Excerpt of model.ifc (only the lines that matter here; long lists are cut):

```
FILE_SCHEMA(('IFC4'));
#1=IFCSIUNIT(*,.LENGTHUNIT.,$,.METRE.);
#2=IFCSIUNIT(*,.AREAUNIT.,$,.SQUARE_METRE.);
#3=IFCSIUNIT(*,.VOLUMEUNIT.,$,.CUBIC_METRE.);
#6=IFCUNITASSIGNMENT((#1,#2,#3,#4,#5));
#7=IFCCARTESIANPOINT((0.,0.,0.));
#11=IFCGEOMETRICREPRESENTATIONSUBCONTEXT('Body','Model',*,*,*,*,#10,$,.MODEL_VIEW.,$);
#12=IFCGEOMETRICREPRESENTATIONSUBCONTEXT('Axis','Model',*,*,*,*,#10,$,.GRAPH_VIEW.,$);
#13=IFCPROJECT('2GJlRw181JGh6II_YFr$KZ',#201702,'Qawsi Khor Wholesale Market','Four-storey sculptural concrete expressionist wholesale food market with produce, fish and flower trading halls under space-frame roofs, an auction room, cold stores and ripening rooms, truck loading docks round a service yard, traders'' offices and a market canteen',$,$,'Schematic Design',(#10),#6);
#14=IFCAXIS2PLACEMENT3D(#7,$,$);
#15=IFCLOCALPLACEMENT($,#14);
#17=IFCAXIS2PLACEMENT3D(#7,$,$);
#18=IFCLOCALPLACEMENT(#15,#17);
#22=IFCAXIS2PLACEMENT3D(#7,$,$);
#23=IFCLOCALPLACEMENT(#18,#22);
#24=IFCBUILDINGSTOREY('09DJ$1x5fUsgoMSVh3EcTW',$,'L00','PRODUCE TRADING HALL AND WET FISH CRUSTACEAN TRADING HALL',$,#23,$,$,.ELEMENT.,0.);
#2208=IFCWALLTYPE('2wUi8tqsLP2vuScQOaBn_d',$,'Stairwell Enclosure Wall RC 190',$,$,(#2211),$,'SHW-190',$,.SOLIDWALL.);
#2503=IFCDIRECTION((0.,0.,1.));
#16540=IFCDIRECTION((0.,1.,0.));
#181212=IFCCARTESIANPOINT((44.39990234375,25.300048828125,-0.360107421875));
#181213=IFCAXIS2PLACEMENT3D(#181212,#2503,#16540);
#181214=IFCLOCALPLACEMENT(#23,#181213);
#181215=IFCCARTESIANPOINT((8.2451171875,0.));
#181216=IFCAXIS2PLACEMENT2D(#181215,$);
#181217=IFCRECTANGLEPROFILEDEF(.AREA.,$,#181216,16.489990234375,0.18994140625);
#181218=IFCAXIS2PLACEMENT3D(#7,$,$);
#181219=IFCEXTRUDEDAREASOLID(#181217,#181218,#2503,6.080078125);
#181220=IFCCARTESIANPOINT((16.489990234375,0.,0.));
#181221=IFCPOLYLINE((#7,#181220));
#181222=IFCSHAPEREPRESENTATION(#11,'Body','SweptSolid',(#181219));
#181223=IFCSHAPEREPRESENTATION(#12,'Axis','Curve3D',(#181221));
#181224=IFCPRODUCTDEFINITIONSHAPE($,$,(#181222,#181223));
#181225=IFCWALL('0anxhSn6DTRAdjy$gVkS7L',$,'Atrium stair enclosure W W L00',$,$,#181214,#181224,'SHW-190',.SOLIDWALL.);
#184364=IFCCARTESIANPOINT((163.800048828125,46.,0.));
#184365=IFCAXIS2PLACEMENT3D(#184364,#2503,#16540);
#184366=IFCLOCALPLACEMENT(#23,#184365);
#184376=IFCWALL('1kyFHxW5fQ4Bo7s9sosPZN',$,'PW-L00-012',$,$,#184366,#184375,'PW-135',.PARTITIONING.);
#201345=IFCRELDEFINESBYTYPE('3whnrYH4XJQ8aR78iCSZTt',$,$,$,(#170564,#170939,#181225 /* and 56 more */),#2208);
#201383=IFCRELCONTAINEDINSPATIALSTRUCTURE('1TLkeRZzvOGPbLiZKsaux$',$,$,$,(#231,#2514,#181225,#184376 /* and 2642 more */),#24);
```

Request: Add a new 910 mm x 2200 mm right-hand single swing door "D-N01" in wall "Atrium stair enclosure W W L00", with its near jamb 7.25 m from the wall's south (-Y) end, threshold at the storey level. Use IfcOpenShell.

```python
import numpy as np
import ifcopenshell
import ifcopenshell.api.feature
import ifcopenshell.api.geometry
import ifcopenshell.api.root
import ifcopenshell.api.spatial
import ifcopenshell.geom
import ifcopenshell.util.element
import ifcopenshell.util.placement
import ifcopenshell.util.representation
import ifcopenshell.util.shape
import ifcopenshell.util.unit

model = ifcopenshell.open("model.ifc")
unit_scale = ifcopenshell.util.unit.calculate_unit_scale(model)
settings = ifcopenshell.geom.settings()


def volume(element):
    """Net volume in cubic metres, openings subtracted."""
    shape = ifcopenshell.geom.create_shape(settings, element)
    return ifcopenshell.util.shape.get_volume(shape.geometry)


wall = model.by_id(181225)
storey = ifcopenshell.util.element.get_container(wall, ifc_class="IfcBuildingStorey")
context = ifcopenshell.util.representation.get_context(model, "Model", "Body", "MODEL_VIEW")
before = volume(wall)

width, height, from_end, sill = 0.91, 2.2, 7.25, 0.0  # metres

# The wall runs along its own X axis, and the end named is its -X end.
wall_shape = ifcopenshell.geom.create_shape(settings, wall)
x, y, z = ifcopenshell.util.shape.get_vertices(wall_shape.geometry).T
start = x.min() + from_end
face, thickness = float(y.min()), float(y.max() - y.min())
wall_matrix = ifcopenshell.util.placement.get_local_placement(wall.ObjectPlacement)
level = ifcopenshell.util.placement.get_local_placement(storey.ObjectPlacement)[2, 3]


def in_wall(x, y):
    """Placement at x, y metres in the wall's axes, at sill height."""
    matrix = wall_matrix.copy()
    matrix[:, 3] = wall_matrix @ np.array([x / unit_scale, y / unit_scale, 0.0, 1.0])
    matrix[2, 3] = level + sill / unit_scale
    return matrix


# Opening: a box that overshoots both wall faces by 50 mm.
opening = ifcopenshell.api.root.create_entity(model, ifc_class="IfcOpeningElement", predefined_type="OPENING")
box = ifcopenshell.api.geometry.add_wall_representation(
    model, context=context, length=width, height=height, thickness=thickness + 0.1
)
ifcopenshell.api.geometry.assign_representation(model, product=opening, representation=box)
ifcopenshell.api.geometry.edit_object_placement(model, product=opening, matrix=in_wall(start, face - 0.05), is_si=False)
ifcopenshell.api.feature.add_feature(model, feature=opening, element=wall)

door = ifcopenshell.api.root.create_entity(model, ifc_class="IfcDoor", name="D-N01", predefined_type="DOOR")
door.OverallWidth, door.OverallHeight = width / unit_scale, height / unit_scale
door.OperationType = "SINGLE_SWING_RIGHT"
body = ifcopenshell.api.geometry.add_door_representation(
    model,
    context=context,
    overall_width=door.OverallWidth,
    overall_height=door.OverallHeight,
    operation_type="SINGLE_SWING_RIGHT",
    lining_properties={"LiningDepth": thickness / unit_scale, "ThresholdDepth": thickness / unit_scale},
)
ifcopenshell.api.geometry.assign_representation(model, product=door, representation=body)
ifcopenshell.api.spatial.assign_container(model, products=[door], relating_structure=storey)
ifcopenshell.api.feature.add_filling(model, opening=opening, element=door)

# The lining spans the wall, so the door starts at the wall face.
ifcopenshell.api.geometry.edit_object_placement(model, product=door, matrix=in_wall(start, face), is_si=False)

after = volume(wall)

print(f"wall volume {before:.3f} -> {after:.3f} m3")

model.write("model-out.ifc")
```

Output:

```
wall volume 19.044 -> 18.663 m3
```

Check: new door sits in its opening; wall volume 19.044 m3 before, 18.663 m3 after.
